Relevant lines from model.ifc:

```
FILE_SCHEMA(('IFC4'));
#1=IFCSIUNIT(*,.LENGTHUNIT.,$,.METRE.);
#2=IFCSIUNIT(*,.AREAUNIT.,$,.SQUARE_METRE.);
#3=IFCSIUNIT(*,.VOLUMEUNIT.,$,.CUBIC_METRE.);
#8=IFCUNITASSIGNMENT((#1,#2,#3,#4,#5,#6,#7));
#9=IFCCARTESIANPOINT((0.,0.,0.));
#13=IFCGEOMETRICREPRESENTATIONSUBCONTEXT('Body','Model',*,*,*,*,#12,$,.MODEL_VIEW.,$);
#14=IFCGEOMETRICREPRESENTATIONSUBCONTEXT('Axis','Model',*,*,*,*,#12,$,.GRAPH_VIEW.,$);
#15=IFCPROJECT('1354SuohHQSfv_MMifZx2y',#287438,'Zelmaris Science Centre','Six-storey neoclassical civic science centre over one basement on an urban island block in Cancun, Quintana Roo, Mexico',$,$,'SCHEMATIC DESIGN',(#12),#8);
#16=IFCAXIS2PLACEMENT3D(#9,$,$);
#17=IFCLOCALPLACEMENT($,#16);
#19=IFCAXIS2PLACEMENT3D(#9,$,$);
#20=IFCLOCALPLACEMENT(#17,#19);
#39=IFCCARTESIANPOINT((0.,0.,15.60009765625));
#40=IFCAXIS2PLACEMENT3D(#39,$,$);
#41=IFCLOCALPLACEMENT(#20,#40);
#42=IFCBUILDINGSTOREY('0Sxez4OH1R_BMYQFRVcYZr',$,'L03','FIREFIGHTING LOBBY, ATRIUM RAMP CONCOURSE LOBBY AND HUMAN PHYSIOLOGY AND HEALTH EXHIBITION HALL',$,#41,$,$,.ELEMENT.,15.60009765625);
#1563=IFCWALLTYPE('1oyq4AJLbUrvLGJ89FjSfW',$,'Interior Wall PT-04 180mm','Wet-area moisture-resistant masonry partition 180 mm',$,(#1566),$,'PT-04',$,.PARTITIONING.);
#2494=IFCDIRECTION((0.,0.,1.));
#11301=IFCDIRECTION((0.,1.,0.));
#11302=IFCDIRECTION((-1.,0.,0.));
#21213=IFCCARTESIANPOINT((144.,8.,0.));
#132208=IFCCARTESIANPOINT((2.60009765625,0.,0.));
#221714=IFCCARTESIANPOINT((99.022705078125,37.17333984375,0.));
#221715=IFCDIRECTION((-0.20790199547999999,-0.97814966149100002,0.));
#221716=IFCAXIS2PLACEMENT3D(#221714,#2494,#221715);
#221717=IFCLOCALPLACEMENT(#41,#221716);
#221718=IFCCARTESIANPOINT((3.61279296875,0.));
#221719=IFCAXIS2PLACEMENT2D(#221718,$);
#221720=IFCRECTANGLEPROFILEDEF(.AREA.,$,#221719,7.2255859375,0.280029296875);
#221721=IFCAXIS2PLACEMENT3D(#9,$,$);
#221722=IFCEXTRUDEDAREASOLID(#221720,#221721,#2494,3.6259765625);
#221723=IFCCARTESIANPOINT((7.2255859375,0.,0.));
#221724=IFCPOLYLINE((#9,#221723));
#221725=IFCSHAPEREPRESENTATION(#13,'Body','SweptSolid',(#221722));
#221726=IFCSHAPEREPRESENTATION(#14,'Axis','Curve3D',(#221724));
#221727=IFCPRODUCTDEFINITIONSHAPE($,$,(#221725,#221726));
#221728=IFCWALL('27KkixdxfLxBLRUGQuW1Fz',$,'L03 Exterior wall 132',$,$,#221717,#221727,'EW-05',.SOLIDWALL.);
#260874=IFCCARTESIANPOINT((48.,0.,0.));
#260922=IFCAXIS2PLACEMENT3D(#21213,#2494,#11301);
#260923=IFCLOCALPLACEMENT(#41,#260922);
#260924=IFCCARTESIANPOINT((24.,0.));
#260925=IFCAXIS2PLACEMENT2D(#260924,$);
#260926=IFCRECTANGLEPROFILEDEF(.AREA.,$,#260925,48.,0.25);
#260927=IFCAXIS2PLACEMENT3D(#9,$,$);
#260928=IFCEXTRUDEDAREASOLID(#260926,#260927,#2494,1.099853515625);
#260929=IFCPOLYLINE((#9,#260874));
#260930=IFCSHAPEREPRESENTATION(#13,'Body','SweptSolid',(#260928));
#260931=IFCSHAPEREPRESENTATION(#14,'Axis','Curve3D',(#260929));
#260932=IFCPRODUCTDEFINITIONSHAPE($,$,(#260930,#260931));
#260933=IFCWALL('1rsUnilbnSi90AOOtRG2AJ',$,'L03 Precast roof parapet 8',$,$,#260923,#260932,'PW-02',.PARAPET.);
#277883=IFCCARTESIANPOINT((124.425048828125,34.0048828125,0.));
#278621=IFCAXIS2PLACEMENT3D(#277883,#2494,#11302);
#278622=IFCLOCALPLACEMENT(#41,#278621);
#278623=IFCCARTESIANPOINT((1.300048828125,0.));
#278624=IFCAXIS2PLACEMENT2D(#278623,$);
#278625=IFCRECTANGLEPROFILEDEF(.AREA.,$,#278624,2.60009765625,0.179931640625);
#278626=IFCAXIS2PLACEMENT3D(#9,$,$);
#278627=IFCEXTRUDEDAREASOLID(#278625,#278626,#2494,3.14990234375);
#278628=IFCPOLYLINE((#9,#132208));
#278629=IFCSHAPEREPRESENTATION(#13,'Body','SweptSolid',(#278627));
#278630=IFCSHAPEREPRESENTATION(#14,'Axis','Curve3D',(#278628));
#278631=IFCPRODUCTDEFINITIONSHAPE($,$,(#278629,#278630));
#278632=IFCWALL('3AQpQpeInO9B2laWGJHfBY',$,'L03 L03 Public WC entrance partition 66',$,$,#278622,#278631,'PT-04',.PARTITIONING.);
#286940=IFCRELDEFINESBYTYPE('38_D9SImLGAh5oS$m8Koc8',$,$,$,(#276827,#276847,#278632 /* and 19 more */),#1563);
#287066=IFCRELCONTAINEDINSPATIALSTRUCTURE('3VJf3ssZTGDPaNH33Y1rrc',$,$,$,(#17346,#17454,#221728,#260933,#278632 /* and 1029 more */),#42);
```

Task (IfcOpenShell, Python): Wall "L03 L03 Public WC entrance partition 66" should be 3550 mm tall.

```python
import ifcopenshell
import ifcopenshell.geom
import ifcopenshell.util.representation
import ifcopenshell.util.shape

model = ifcopenshell.open("model.ifc")
settings = ifcopenshell.geom.settings()


def volume(element):
    """Net volume in cubic metres, openings subtracted."""
    shape = ifcopenshell.geom.create_shape(settings, element)
    return ifcopenshell.util.shape.get_volume(shape.geometry)


wall = model.by_guid("3AQpQpeInO9B2laWGJHfBY")
before = volume(wall)

body = ifcopenshell.util.representation.get_representation(wall, "Model", "Body")
solid = body.Items[0]
old_height = solid.Depth
solid.Depth = 3.55
after = volume(wall)

print(f"height {old_height:g} -> {solid.Depth:g}, volume {before:.3f} -> {after:.3f} m3")

model.write("model_rev.ifc")
```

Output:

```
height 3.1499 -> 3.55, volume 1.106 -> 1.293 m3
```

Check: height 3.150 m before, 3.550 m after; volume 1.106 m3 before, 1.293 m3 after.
